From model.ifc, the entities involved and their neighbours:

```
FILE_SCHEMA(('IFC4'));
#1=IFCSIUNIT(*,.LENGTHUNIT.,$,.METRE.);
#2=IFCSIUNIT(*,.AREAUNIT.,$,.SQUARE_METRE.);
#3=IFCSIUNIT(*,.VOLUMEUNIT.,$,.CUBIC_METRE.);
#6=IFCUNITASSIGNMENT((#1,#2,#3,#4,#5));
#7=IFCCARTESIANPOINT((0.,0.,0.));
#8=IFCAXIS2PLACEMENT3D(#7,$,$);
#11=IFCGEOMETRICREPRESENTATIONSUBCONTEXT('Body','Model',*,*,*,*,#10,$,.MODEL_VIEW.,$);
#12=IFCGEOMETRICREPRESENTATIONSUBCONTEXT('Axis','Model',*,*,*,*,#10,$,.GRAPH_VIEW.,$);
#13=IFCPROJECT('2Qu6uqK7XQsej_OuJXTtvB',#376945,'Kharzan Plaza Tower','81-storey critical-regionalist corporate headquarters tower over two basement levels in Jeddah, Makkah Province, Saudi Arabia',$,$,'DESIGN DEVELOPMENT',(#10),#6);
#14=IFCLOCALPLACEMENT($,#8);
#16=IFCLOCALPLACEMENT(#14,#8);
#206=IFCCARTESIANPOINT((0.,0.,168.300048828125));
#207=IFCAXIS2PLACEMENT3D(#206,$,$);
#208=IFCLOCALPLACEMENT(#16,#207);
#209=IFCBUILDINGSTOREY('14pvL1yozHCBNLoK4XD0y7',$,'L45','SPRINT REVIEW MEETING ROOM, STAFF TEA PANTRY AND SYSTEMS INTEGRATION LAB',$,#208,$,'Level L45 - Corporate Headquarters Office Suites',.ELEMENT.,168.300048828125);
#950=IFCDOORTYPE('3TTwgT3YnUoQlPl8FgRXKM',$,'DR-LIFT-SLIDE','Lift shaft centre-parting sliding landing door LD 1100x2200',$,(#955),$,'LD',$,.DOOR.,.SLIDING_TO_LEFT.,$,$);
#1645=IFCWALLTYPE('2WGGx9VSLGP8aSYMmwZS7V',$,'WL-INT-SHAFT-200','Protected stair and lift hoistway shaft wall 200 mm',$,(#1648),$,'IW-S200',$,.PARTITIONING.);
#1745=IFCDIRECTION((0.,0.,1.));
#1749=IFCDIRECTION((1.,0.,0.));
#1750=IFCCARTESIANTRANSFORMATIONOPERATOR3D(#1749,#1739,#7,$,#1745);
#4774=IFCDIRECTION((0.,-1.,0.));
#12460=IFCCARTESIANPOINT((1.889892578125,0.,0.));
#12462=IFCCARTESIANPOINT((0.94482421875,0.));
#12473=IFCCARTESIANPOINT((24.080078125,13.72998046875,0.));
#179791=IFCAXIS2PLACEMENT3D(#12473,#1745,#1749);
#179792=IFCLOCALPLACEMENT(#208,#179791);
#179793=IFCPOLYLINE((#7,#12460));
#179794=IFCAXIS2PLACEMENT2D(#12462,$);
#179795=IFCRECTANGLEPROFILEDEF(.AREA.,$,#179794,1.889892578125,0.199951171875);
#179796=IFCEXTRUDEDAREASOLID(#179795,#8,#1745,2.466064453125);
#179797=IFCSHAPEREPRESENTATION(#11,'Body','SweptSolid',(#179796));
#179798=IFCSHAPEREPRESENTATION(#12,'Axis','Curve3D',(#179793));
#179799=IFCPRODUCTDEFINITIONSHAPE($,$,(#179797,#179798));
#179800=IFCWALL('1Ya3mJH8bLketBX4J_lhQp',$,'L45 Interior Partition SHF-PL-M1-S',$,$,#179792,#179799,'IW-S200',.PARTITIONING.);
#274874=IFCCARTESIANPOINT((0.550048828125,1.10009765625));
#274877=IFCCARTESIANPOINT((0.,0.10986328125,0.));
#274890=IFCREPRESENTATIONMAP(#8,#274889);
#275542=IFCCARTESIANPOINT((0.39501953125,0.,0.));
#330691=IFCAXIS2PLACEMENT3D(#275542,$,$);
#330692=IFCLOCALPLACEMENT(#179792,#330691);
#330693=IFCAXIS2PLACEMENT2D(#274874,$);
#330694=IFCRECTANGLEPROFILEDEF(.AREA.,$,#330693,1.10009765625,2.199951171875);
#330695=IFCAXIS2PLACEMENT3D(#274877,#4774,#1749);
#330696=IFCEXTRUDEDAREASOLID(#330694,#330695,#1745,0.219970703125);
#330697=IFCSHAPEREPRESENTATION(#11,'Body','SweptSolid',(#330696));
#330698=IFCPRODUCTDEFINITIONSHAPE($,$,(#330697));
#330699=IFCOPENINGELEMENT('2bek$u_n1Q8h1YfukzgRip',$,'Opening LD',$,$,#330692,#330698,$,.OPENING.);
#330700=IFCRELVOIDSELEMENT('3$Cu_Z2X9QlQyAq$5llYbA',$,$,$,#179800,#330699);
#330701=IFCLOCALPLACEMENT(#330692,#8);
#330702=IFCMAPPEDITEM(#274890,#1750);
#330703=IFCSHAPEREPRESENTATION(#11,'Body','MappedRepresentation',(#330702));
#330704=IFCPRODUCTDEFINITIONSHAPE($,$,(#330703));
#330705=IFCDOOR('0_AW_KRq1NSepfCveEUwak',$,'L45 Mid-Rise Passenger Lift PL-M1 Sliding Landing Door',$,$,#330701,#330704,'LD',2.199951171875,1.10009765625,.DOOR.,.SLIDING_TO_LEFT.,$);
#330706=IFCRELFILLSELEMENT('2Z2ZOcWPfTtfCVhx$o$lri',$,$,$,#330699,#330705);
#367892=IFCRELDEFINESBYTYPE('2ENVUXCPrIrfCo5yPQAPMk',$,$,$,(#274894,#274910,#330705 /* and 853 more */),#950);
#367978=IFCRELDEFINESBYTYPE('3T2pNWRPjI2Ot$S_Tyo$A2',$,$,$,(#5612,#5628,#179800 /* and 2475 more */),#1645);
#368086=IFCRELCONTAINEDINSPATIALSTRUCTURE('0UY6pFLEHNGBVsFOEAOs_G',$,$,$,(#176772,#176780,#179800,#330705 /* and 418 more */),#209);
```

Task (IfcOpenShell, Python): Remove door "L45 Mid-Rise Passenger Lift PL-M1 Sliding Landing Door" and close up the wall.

```python
import ifcopenshell
import ifcopenshell.api.feature
import ifcopenshell.api.root
import ifcopenshell.geom
import ifcopenshell.util.shape

model = ifcopenshell.open("model.ifc")
settings = ifcopenshell.geom.settings()


def volume(element):
    """Net volume in cubic metres, openings subtracted."""
    shape = ifcopenshell.geom.create_shape(settings, element)
    return ifcopenshell.util.shape.get_volume(shape.geometry)


door = model.by_guid("0_AW_KRq1NSepfCveEUwak")
opening = door.FillsVoids[0].RelatingOpeningElement
wall = opening.VoidsElements[0].RelatingBuildingElement
before = volume(wall)

ifcopenshell.api.root.remove_product(model, product=door)
ifcopenshell.api.feature.remove_feature(model, feature=opening)

after = volume(wall)

print(f"wall volume {before:.3f} -> {after:.3f} m3")

model.write("model_updated.ifc")
```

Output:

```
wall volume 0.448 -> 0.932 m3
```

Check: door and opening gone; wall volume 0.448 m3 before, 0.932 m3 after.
